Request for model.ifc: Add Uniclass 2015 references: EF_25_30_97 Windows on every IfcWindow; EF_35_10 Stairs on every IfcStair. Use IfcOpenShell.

First a look at what the model holds.

```python
import ifcopenshell

model = ifcopenshell.open("model.ifc")
print(model.schema)
print("classifications:", [c.Name for c in model.by_type("IfcClassification")])
for ifc_class in ("IfcDoor", "IfcRoof", "IfcStair", "IfcWall", "IfcWindow"):
    print(ifc_class, len(model.by_type(ifc_class)))
```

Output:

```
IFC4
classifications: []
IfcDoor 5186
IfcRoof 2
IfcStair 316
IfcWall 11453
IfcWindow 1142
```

```python
import ifcopenshell
import ifcopenshell.api.classification

model = ifcopenshell.open("model.ifc")

system = ifcopenshell.api.classification.add_classification(model, classification="Uniclass 2015")

codes = {
    "IfcWindow": ("EF_25_30_97", "Windows"),
    "IfcStair": ("EF_35_10", "Stairs"),
}
for ifc_class, (code, name) in codes.items():
    products = model.by_type(ifc_class)
    ifcopenshell.api.classification.add_reference(
        model, products=products, classification=system, identification=code, name=name
    )
    print(code, len(products))

model.write("model-out.ifc")
```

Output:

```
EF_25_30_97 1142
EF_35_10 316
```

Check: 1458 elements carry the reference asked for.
